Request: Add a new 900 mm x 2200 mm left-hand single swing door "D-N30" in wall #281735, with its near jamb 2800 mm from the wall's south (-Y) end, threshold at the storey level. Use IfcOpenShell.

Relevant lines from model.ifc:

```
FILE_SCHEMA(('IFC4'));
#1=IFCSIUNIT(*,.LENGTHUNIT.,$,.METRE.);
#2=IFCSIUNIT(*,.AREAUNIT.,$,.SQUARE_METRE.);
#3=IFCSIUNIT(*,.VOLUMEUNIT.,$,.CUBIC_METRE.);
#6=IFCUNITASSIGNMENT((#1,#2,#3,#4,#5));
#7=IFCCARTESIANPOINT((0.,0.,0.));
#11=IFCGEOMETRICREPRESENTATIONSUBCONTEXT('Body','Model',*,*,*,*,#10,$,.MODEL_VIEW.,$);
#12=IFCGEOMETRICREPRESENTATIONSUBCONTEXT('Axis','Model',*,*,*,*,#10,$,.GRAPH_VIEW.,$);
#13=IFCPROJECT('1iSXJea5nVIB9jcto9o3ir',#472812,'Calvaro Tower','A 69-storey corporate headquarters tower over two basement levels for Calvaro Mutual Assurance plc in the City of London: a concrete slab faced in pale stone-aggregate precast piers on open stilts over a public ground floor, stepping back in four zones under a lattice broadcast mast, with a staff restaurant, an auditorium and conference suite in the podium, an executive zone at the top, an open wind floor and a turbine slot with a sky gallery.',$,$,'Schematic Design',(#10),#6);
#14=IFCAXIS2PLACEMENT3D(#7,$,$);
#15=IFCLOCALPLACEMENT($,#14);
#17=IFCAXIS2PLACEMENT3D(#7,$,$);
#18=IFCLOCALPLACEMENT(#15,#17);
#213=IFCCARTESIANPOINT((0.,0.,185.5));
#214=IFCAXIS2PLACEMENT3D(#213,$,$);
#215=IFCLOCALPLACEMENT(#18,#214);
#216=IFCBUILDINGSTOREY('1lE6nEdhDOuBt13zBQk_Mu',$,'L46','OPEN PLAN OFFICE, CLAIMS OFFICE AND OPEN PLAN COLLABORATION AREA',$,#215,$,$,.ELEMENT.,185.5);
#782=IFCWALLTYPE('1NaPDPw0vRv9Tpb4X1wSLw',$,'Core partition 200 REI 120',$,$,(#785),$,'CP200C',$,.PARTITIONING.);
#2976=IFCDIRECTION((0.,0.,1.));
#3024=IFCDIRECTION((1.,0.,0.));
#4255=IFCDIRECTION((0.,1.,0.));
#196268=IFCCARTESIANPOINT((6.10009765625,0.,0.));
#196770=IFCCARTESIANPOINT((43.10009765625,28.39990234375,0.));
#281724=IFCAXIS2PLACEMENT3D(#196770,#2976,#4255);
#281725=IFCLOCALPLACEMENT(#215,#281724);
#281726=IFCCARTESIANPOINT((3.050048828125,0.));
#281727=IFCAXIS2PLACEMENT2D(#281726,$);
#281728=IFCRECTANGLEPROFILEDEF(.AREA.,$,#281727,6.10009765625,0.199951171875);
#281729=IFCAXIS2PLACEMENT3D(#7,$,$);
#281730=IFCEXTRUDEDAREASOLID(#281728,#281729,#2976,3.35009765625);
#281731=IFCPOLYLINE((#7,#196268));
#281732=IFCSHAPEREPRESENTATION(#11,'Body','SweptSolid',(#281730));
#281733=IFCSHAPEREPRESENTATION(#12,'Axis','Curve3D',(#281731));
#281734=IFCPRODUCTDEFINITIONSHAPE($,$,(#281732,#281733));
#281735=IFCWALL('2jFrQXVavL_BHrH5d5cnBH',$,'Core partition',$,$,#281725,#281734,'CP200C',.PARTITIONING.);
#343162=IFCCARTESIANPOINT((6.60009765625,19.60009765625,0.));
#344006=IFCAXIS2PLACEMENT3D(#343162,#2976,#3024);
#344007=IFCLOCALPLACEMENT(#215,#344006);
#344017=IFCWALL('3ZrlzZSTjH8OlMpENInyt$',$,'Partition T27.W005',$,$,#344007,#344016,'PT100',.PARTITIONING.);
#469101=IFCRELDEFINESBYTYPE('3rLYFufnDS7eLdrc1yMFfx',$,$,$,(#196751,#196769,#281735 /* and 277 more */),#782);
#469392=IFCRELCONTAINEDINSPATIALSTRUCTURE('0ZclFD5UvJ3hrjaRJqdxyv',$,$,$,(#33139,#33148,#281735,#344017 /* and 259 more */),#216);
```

```python
import numpy as np
import ifcopenshell
import ifcopenshell.api.feature
import ifcopenshell.api.geometry
import ifcopenshell.api.root
import ifcopenshell.api.spatial
import ifcopenshell.geom
import ifcopenshell.util.element
import ifcopenshell.util.placement
import ifcopenshell.util.representation
import ifcopenshell.util.shape
import ifcopenshell.util.unit

model = ifcopenshell.open("model.ifc")
unit_scale = ifcopenshell.util.unit.calculate_unit_scale(model)
settings = ifcopenshell.geom.settings()


def volume(element):
    """Net volume in cubic metres, openings subtracted."""
    shape = ifcopenshell.geom.create_shape(settings, element)
    return ifcopenshell.util.shape.get_volume(shape.geometry)


wall = model.by_guid("2jFrQXVavL_BHrH5d5cnBH")
storey = ifcopenshell.util.element.get_container(wall, ifc_class="IfcBuildingStorey")
context = ifcopenshell.util.representation.get_context(model, "Model", "Body", "MODEL_VIEW")
before = volume(wall)

width, height, from_end, sill = 0.9, 2.2, 2.8, 0.0  # metres

# The wall runs along its own X axis, and the end named is its -X end.
wall_shape = ifcopenshell.geom.create_shape(settings, wall)
x, y, z = ifcopenshell.util.shape.get_vertices(wall_shape.geometry).T
start = x.min() + from_end
face, thickness = float(y.min()), float(y.max() - y.min())
wall_matrix = ifcopenshell.util.placement.get_local_placement(wall.ObjectPlacement)
level = ifcopenshell.util.placement.get_local_placement(storey.ObjectPlacement)[2, 3]


def in_wall(x, y):
    """Placement at x, y metres in the wall's axes, at sill height."""
    matrix = wall_matrix.copy()
    matrix[:, 3] = wall_matrix @ np.array([x / unit_scale, y / unit_scale, 0.0, 1.0])
    matrix[2, 3] = level + sill / unit_scale
    return matrix


# Opening: a box that overshoots both wall faces by 50 mm.
opening = ifcopenshell.api.root.create_entity(model, ifc_class="IfcOpeningElement", predefined_type="OPENING")
box = ifcopenshell.api.geometry.add_wall_representation(
    model, context=context, length=width, height=height, thickness=thickness + 0.1
)
ifcopenshell.api.geometry.assign_representation(model, product=opening, representation=box)
ifcopenshell.api.geometry.edit_object_placement(model, product=opening, matrix=in_wall(start, face - 0.05), is_si=False)
ifcopenshell.api.feature.add_feature(model, feature=opening, element=wall)

door = ifcopenshell.api.root.create_entity(model, ifc_class="IfcDoor", name="D-N30", predefined_type="DOOR")
door.OverallWidth, door.OverallHeight = width / unit_scale, height / unit_scale
door.OperationType = "SINGLE_SWING_LEFT"
body = ifcopenshell.api.geometry.add_door_representation(
    model,
    context=context,
    overall_width=door.OverallWidth,
    overall_height=door.OverallHeight,
    operation_type="SINGLE_SWING_LEFT",
    lining_properties={"LiningDepth": thickness / unit_scale, "ThresholdDepth": thickness / unit_scale},
)
ifcopenshell.api.geometry.assign_representation(model, product=door, representation=body)
ifcopenshell.api.spatial.assign_container(model, products=[door], relating_structure=storey)
ifcopenshell.api.feature.add_filling(model, opening=opening, element=door)

# The lining spans the wall, so the door starts at the wall face.
ifcopenshell.api.geometry.edit_object_placement(model, product=door, matrix=in_wall(start, face), is_si=False)

after = volume(wall)

print(f"wall volume {before:.3f} -> {after:.3f} m3")

model.write("model_v2.ifc")
```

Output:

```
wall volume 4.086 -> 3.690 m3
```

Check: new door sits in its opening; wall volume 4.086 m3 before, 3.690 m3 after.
